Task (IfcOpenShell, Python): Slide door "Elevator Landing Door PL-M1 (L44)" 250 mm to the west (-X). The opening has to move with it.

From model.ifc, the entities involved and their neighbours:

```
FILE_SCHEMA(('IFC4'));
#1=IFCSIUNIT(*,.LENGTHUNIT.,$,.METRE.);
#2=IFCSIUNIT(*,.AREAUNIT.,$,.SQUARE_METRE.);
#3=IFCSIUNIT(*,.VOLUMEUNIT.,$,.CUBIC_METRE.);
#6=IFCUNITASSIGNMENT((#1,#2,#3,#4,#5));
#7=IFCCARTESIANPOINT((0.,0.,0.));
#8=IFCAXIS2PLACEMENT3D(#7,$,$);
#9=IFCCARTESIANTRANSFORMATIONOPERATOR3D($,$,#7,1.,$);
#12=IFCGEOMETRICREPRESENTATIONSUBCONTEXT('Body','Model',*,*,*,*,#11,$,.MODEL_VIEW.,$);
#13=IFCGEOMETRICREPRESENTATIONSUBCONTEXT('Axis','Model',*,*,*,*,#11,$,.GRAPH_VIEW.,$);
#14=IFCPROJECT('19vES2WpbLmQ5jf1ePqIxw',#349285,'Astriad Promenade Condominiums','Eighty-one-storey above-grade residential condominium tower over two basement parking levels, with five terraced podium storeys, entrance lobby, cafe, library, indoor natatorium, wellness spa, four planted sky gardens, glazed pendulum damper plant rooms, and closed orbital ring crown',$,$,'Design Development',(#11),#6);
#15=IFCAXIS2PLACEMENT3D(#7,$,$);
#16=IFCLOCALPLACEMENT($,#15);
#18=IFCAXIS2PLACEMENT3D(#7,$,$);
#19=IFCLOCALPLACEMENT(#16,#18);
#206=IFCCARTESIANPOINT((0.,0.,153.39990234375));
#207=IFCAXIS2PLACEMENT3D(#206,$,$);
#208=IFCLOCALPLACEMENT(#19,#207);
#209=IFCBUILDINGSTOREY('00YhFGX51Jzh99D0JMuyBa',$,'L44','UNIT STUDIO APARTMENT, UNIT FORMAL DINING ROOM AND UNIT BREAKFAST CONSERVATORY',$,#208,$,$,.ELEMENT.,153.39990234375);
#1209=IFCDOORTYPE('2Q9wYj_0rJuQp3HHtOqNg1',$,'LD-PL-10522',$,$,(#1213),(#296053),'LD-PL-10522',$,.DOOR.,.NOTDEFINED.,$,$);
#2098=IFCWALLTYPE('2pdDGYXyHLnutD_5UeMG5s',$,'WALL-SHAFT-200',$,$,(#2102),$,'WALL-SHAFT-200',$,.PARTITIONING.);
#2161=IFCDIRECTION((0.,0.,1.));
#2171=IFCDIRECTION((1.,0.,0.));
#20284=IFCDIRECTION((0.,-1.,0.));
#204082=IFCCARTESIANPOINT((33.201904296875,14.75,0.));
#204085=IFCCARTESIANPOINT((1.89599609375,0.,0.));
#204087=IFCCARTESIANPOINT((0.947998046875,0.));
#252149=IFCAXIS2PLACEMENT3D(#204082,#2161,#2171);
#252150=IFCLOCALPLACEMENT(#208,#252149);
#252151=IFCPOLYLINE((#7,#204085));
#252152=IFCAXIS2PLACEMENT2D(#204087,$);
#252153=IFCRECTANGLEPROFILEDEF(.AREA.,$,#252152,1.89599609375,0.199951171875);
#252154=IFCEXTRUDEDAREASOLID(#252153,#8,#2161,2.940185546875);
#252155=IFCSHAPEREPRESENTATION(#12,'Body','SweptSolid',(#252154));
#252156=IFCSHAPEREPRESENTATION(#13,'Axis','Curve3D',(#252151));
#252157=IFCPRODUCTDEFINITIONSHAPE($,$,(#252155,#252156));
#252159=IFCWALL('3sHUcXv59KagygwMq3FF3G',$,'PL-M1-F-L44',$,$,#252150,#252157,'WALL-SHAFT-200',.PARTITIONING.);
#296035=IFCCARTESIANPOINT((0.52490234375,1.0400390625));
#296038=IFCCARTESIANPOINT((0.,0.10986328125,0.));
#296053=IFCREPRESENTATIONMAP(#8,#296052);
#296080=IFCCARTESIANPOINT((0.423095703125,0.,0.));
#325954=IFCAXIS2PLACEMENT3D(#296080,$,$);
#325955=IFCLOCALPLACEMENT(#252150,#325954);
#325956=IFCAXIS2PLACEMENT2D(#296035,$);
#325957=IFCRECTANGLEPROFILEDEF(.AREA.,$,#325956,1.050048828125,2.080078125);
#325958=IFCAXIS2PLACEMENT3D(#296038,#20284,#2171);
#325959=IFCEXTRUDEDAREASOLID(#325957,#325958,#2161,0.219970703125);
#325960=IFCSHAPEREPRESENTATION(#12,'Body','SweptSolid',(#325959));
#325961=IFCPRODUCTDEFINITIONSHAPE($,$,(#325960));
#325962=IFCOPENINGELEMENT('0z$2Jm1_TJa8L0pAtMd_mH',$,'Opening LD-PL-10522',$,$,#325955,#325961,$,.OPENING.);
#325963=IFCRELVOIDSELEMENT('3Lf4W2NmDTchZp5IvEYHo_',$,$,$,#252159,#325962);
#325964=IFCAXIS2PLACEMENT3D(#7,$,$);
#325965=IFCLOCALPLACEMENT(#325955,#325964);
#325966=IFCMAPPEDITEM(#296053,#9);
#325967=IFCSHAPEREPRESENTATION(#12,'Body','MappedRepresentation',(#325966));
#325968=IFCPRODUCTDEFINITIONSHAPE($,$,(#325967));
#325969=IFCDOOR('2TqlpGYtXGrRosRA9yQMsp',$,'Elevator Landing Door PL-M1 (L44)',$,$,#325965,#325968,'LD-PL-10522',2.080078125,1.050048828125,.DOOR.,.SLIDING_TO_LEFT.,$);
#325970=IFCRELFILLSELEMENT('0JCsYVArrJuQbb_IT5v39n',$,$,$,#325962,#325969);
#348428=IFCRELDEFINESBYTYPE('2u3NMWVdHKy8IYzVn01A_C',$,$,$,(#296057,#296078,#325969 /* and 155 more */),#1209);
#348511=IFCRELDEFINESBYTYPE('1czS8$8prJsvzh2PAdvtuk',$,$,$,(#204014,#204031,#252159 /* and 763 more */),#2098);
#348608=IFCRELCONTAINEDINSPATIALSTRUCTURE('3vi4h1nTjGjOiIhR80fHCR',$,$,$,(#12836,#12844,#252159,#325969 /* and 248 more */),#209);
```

```python
import ifcopenshell
import ifcopenshell.api.geometry
import ifcopenshell.util.placement
import ifcopenshell.util.unit

model = ifcopenshell.open("model.ifc")
unit_scale = ifcopenshell.util.unit.calculate_unit_scale(model)

door = model.by_guid("2TqlpGYtXGrRosRA9yQMsp")
opening = door.FillsVoids[0].RelatingOpeningElement
wall = opening.VoidsElements[0].RelatingBuildingElement

wall_matrix = ifcopenshell.util.placement.get_local_placement(wall.ObjectPlacement)
shift = wall_matrix[:3, 0] * -0.25 / unit_scale
before = ifcopenshell.util.placement.get_local_placement(door.ObjectPlacement)[:3, 3].copy()

# The door is placed relative to its opening, so it follows when the opening moves.
matrix = ifcopenshell.util.placement.get_local_placement(opening.ObjectPlacement)
matrix[:3, 3] += shift
ifcopenshell.api.geometry.edit_object_placement(
    model, product=opening, matrix=matrix, is_si=False, should_transform_children=True
)

after = ifcopenshell.util.placement.get_local_placement(door.ObjectPlacement)[:3, 3]
print("door moved by", (after - before).round(3) + 0.0)

model.write("model_updated.ifc")
```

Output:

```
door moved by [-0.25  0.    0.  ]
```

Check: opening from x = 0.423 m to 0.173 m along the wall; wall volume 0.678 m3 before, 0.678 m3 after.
